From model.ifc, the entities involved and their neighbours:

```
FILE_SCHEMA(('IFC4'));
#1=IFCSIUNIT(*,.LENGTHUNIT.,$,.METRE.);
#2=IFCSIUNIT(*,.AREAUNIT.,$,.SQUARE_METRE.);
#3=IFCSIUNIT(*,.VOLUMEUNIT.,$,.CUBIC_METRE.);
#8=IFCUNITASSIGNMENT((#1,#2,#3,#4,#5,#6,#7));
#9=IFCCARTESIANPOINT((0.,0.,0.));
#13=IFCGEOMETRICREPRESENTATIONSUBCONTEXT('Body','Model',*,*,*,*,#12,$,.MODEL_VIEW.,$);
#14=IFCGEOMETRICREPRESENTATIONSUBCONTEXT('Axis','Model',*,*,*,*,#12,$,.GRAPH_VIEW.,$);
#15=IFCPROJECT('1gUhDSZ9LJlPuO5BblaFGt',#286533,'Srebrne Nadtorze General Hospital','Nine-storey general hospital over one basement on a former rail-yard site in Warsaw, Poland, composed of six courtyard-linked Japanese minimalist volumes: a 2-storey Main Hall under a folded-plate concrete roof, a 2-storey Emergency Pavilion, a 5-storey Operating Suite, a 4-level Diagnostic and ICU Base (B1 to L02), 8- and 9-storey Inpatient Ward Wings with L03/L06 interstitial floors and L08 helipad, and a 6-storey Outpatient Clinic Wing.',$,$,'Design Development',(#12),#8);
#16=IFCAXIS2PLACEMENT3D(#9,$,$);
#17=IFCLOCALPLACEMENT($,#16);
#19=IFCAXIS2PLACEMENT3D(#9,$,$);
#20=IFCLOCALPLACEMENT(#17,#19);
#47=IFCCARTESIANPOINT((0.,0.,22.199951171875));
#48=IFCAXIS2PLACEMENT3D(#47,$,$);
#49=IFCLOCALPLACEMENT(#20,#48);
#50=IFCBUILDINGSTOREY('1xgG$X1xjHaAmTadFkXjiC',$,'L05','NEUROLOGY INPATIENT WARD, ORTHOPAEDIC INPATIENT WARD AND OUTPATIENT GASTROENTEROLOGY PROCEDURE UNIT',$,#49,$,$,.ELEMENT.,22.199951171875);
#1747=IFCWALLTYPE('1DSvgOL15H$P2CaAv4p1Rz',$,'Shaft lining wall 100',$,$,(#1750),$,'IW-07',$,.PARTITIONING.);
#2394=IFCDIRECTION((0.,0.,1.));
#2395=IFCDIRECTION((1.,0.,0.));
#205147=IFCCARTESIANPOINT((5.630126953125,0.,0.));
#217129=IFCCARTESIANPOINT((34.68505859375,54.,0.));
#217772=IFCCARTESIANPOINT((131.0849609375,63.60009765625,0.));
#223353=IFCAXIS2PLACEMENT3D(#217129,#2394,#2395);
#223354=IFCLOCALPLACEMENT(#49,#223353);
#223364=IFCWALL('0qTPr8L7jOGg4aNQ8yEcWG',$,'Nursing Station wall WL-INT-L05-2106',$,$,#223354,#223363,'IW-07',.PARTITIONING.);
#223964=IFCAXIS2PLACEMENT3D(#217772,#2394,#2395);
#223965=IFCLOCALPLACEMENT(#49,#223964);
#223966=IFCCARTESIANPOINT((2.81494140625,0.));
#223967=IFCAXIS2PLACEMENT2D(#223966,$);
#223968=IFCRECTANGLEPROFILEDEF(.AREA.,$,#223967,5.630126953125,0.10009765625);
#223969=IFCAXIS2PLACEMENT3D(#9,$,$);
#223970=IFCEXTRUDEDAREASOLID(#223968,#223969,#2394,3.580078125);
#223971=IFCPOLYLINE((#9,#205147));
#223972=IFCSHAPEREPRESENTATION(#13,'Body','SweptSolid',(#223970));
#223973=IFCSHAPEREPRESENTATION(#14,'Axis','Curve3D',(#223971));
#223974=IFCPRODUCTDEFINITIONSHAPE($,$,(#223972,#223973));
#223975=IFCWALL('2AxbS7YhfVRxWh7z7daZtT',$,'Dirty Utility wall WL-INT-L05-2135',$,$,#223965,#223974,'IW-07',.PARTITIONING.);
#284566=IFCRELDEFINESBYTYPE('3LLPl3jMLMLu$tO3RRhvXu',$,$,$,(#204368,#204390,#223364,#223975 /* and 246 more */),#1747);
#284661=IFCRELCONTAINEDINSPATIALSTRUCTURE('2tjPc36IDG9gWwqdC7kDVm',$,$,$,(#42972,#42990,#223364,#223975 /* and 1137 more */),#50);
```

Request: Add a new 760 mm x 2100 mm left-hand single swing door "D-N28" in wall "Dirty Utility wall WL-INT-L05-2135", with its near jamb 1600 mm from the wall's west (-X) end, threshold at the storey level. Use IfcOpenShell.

```python
import numpy as np
import ifcopenshell
import ifcopenshell.api.feature
import ifcopenshell.api.geometry
import ifcopenshell.api.root
import ifcopenshell.api.spatial
import ifcopenshell.geom
import ifcopenshell.util.element
import ifcopenshell.util.placement
import ifcopenshell.util.representation
import ifcopenshell.util.shape
import ifcopenshell.util.unit

model = ifcopenshell.open("model.ifc")
unit_scale = ifcopenshell.util.unit.calculate_unit_scale(model)
settings = ifcopenshell.geom.settings()


def volume(element):
    """Net volume in cubic metres, openings subtracted."""
    shape = ifcopenshell.geom.create_shape(settings, element)
    return ifcopenshell.util.shape.get_volume(shape.geometry)


wall = model.by_id(223975)
storey = ifcopenshell.util.element.get_container(wall, ifc_class="IfcBuildingStorey")
context = ifcopenshell.util.representation.get_context(model, "Model", "Body", "MODEL_VIEW")
before = volume(wall)

width, height, from_end, sill = 0.76, 2.1, 1.6, 0.0  # metres

# The wall runs along its own X axis, and the end named is its -X end.
wall_shape = ifcopenshell.geom.create_shape(settings, wall)
x, y, z = ifcopenshell.util.shape.get_vertices(wall_shape.geometry).T
start = x.min() + from_end
face, thickness = float(y.min()), float(y.max() - y.min())
wall_matrix = ifcopenshell.util.placement.get_local_placement(wall.ObjectPlacement)
level = ifcopenshell.util.placement.get_local_placement(storey.ObjectPlacement)[2, 3]


def in_wall(x, y):
    """Placement at x, y metres in the wall's axes, at sill height."""
    matrix = wall_matrix.copy()
    matrix[:, 3] = wall_matrix @ np.array([x / unit_scale, y / unit_scale, 0.0, 1.0])
    matrix[2, 3] = level + sill / unit_scale
    return matrix


# Opening: a box that overshoots both wall faces by 50 mm.
opening = ifcopenshell.api.root.create_entity(model, ifc_class="IfcOpeningElement", predefined_type="OPENING")
box = ifcopenshell.api.geometry.add_wall_representation(
    model, context=context, length=width, height=height, thickness=thickness + 0.1
)
ifcopenshell.api.geometry.assign_representation(model, product=opening, representation=box)
ifcopenshell.api.geometry.edit_object_placement(model, product=opening, matrix=in_wall(start, face - 0.05), is_si=False)
ifcopenshell.api.feature.add_feature(model, feature=opening, element=wall)

door = ifcopenshell.api.root.create_entity(model, ifc_class="IfcDoor", name="D-N28", predefined_type="DOOR")
door.OverallWidth, door.OverallHeight = width / unit_scale, height / unit_scale
door.OperationType = "SINGLE_SWING_LEFT"
body = ifcopenshell.api.geometry.add_door_representation(
    model,
    context=context,
    overall_width=door.OverallWidth,
    overall_height=door.OverallHeight,
    operation_type="SINGLE_SWING_LEFT",
    lining_properties={"LiningDepth": thickness / unit_scale, "ThresholdDepth": thickness / unit_scale},
)
ifcopenshell.api.geometry.assign_representation(model, product=door, representation=body)
ifcopenshell.api.spatial.assign_container(model, products=[door], relating_structure=storey)
ifcopenshell.api.feature.add_filling(model, opening=opening, element=door)

# The lining spans the wall, so the door starts at the wall face.
ifcopenshell.api.geometry.edit_object_placement(model, product=door, matrix=in_wall(start, face), is_si=False)

after = volume(wall)

print(f"wall volume {before:.3f} -> {after:.3f} m3")

model.write("model-out.ifc")
```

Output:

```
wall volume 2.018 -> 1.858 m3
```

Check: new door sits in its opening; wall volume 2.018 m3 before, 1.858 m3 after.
